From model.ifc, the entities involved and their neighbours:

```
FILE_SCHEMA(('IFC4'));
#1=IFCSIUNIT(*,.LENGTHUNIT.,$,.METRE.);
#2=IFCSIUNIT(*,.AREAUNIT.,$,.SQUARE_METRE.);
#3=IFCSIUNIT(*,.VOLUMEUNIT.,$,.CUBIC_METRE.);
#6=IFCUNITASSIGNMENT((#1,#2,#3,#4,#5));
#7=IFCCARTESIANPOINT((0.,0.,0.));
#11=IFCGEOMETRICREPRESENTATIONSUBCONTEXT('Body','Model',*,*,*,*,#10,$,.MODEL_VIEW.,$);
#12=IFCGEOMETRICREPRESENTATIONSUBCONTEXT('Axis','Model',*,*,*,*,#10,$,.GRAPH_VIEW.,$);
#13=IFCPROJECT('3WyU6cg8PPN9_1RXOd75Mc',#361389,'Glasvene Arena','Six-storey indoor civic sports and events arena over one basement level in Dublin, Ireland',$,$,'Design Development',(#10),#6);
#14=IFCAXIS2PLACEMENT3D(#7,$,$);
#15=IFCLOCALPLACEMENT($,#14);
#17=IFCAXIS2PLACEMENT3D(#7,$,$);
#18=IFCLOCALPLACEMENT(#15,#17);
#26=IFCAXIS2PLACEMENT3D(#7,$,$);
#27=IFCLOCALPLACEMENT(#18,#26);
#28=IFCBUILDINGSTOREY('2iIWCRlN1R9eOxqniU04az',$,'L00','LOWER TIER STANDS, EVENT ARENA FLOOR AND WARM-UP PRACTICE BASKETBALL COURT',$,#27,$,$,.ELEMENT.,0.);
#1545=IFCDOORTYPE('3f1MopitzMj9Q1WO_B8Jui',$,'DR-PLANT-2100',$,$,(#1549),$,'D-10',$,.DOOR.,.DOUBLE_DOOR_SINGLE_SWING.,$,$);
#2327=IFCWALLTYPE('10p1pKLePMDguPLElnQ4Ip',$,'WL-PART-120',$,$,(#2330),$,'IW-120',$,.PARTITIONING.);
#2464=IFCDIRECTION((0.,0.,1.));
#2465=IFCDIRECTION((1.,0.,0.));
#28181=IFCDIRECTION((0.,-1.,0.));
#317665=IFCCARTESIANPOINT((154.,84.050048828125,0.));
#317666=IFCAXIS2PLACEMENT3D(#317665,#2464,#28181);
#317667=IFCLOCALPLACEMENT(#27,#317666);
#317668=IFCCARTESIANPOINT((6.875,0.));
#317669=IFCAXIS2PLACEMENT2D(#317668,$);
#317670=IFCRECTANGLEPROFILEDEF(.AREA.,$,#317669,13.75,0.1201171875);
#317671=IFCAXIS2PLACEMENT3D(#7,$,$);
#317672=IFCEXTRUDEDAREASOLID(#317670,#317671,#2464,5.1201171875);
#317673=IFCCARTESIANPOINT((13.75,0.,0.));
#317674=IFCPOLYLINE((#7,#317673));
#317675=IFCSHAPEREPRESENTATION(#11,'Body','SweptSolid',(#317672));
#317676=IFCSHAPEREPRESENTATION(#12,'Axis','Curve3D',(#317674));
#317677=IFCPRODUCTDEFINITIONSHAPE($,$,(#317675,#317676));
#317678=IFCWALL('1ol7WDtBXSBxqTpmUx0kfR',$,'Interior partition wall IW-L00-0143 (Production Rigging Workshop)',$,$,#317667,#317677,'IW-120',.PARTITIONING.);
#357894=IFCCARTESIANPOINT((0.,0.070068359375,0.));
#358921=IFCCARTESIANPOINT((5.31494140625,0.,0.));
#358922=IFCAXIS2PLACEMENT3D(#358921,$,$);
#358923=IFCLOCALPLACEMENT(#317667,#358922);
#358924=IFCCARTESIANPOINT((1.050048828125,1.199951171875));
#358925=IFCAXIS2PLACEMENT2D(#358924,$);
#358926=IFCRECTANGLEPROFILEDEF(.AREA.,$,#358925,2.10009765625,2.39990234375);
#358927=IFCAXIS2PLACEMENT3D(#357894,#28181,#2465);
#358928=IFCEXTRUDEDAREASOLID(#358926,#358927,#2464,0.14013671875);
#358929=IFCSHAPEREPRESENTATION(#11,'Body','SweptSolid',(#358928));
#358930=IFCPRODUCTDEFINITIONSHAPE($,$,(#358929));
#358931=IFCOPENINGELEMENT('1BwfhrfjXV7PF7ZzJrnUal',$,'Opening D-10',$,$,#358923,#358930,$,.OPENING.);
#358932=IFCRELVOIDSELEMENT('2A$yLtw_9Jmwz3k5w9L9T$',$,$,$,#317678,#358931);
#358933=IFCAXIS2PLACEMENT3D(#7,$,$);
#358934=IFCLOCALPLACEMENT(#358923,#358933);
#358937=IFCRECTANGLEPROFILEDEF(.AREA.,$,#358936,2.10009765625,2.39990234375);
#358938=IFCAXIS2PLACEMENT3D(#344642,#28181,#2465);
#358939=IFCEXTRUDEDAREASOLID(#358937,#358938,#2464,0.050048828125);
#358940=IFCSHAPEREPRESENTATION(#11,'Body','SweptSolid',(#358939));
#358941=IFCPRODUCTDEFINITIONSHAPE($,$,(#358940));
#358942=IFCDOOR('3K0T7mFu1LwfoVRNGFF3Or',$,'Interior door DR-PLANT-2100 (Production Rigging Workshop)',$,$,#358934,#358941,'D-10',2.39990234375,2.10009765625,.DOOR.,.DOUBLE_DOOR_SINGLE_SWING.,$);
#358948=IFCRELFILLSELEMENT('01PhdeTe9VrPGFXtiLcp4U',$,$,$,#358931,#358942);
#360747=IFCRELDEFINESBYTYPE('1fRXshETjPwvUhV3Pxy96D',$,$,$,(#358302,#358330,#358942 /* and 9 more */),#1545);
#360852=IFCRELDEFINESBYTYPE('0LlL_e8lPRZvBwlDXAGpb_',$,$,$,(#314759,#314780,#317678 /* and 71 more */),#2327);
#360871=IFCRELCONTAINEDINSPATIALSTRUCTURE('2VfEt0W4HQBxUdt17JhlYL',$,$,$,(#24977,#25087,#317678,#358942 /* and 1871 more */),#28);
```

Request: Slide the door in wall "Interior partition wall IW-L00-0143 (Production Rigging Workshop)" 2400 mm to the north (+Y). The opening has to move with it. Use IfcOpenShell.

```python
import ifcopenshell
import ifcopenshell.api.geometry
import ifcopenshell.util.placement

model = ifcopenshell.open("model.ifc")

door = model.by_guid("3K0T7mFu1LwfoVRNGFF3Or")
opening = door.FillsVoids[0].RelatingOpeningElement
wall = opening.VoidsElements[0].RelatingBuildingElement

wall_matrix = ifcopenshell.util.placement.get_local_placement(wall.ObjectPlacement)
shift = wall_matrix[:3, 0] * -2.4
before = ifcopenshell.util.placement.get_local_placement(door.ObjectPlacement)[:3, 3].copy()

# The door is placed relative to its opening, so it follows when the opening moves.
matrix = ifcopenshell.util.placement.get_local_placement(opening.ObjectPlacement)
matrix[:3, 3] += shift
ifcopenshell.api.geometry.edit_object_placement(
    model, product=opening, matrix=matrix, is_si=False, should_transform_children=True
)

after = ifcopenshell.util.placement.get_local_placement(door.ObjectPlacement)[:3, 3]
print("door moved by", (after - before).round(3) + 0.0)

model.write("model_v2.ifc")
```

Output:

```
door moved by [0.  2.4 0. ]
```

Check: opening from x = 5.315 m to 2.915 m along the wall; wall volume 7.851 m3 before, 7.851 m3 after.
